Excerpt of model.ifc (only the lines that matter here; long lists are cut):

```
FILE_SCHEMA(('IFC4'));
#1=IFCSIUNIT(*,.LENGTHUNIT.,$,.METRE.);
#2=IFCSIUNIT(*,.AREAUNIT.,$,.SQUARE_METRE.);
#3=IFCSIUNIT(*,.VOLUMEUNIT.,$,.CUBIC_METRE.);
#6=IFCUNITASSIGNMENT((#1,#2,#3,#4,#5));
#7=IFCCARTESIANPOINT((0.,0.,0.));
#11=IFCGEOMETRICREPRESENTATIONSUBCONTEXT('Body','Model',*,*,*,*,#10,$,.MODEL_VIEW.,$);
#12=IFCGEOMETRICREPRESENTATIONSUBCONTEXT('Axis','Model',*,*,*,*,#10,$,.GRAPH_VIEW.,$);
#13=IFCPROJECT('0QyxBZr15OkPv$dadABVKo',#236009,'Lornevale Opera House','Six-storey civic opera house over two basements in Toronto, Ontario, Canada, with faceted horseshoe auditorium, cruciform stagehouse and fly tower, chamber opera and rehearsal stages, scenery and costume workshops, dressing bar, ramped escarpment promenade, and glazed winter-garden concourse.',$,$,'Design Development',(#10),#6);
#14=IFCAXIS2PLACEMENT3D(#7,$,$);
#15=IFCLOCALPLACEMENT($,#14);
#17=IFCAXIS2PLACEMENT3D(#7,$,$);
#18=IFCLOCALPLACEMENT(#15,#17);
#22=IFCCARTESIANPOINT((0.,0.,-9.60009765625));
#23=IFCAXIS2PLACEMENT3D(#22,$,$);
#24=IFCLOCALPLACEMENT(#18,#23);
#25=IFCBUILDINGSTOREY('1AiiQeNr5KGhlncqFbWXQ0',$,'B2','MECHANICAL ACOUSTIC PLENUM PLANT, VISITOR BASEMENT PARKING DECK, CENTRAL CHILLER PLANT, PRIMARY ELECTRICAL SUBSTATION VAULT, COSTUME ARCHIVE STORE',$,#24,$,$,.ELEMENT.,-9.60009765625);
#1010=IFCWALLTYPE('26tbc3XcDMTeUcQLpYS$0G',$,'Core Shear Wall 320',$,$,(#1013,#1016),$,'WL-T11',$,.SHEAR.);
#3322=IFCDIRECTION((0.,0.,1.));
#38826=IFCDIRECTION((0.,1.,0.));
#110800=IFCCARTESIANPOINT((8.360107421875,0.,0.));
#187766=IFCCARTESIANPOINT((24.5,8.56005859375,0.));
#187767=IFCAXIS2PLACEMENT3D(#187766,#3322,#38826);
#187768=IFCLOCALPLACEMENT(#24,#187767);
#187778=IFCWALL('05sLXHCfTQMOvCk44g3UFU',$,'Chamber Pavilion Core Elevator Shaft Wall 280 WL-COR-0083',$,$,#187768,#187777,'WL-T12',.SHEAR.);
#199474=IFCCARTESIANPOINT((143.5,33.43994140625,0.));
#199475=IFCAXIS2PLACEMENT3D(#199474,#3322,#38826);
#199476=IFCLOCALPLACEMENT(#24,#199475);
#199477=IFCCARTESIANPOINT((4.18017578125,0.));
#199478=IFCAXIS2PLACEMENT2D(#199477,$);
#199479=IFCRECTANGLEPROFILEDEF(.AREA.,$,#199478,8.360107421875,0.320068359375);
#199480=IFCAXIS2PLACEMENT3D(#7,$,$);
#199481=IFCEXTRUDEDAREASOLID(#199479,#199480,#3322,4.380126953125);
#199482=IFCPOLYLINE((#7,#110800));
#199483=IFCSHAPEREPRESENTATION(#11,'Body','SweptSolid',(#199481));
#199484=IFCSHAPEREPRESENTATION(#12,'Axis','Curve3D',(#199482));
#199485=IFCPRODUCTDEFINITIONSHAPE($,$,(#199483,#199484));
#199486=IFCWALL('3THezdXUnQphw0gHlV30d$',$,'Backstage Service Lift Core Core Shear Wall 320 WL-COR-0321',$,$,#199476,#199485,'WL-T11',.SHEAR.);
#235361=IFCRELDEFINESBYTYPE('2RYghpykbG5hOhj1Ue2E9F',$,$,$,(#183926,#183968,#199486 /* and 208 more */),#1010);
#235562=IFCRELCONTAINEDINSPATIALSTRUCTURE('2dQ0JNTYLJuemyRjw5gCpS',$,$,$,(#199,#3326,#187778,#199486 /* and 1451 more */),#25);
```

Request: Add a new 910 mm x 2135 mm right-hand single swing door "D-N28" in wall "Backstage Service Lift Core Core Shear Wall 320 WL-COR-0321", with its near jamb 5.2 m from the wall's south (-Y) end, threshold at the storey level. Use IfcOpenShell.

```python
import numpy as np
import ifcopenshell
import ifcopenshell.api.feature
import ifcopenshell.api.geometry
import ifcopenshell.api.root
import ifcopenshell.api.spatial
import ifcopenshell.geom
import ifcopenshell.util.element
import ifcopenshell.util.placement
import ifcopenshell.util.representation
import ifcopenshell.util.shape
import ifcopenshell.util.unit

model = ifcopenshell.open("model.ifc")
unit_scale = ifcopenshell.util.unit.calculate_unit_scale(model)
settings = ifcopenshell.geom.settings()


def volume(element):
    """Net volume in cubic metres, openings subtracted."""
    shape = ifcopenshell.geom.create_shape(settings, element)
    return ifcopenshell.util.shape.get_volume(shape.geometry)


wall = model.by_guid("3THezdXUnQphw0gHlV30d$")
storey = ifcopenshell.util.element.get_container(wall, ifc_class="IfcBuildingStorey")
context = ifcopenshell.util.representation.get_context(model, "Model", "Body", "MODEL_VIEW")
before = volume(wall)

width, height, from_end, sill = 0.91, 2.135, 5.2, 0.0  # metres

# The wall runs along its own X axis, and the end named is its -X end.
wall_shape = ifcopenshell.geom.create_shape(settings, wall)
x, y, z = ifcopenshell.util.shape.get_vertices(wall_shape.geometry).T
start = x.min() + from_end
face, thickness = float(y.min()), float(y.max() - y.min())
wall_matrix = ifcopenshell.util.placement.get_local_placement(wall.ObjectPlacement)
level = ifcopenshell.util.placement.get_local_placement(storey.ObjectPlacement)[2, 3]


def in_wall(x, y):
    """Placement at x, y metres in the wall's axes, at sill height."""
    matrix = wall_matrix.copy()
    matrix[:, 3] = wall_matrix @ np.array([x / unit_scale, y / unit_scale, 0.0, 1.0])
    matrix[2, 3] = level + sill / unit_scale
    return matrix


# Opening: a box that overshoots both wall faces by 50 mm.
opening = ifcopenshell.api.root.create_entity(model, ifc_class="IfcOpeningElement", predefined_type="OPENING")
box = ifcopenshell.api.geometry.add_wall_representation(
    model, context=context, length=width, height=height, thickness=thickness + 0.1
)
ifcopenshell.api.geometry.assign_representation(model, product=opening, representation=box)
ifcopenshell.api.geometry.edit_object_placement(model, product=opening, matrix=in_wall(start, face - 0.05), is_si=False)
ifcopenshell.api.feature.add_feature(model, feature=opening, element=wall)

door = ifcopenshell.api.root.create_entity(model, ifc_class="IfcDoor", name="D-N28", predefined_type="DOOR")
door.OverallWidth, door.OverallHeight = width / unit_scale, height / unit_scale
door.OperationType = "SINGLE_SWING_RIGHT"
body = ifcopenshell.api.geometry.add_door_representation(
    model,
    context=context,
    overall_width=door.OverallWidth,
    overall_height=door.OverallHeight,
    operation_type="SINGLE_SWING_RIGHT",
    lining_properties={"LiningDepth": thickness / unit_scale, "ThresholdDepth": thickness / unit_scale},
)
ifcopenshell.api.geometry.assign_representation(model, product=door, representation=body)
ifcopenshell.api.spatial.assign_container(model, products=[door], relating_structure=storey)
ifcopenshell.api.feature.add_filling(model, opening=opening, element=door)

# The lining spans the wall, so the door starts at the wall face.
ifcopenshell.api.geometry.edit_object_placement(model, product=door, matrix=in_wall(start, face), is_si=False)

after = volume(wall)

print(f"wall volume {before:.3f} -> {after:.3f} m3")

model.write("model-out.ifc")
```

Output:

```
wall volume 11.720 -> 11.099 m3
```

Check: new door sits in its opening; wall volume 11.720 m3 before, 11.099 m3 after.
